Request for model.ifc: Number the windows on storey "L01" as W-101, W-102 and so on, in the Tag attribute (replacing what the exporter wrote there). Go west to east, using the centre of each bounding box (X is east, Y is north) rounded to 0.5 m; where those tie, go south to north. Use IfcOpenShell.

First a look at what the model holds.

```python
import ifcopenshell
import ifcopenshell.util.element
import ifcopenshell.util.placement

model = ifcopenshell.open("model.ifc")
print(model.schema)
storey = next(s for s in model.by_type("IfcBuildingStorey") if s.Name == "L01")
windows = [e for e in ifcopenshell.util.element.get_decomposition(storey) if e.is_a("IfcWindow")]
for e in sorted(windows, key=lambda e: e.id()):
    origin = ifcopenshell.util.placement.get_local_placement(e.ObjectPlacement)[:3, 3]
    print(e.id(), e.Tag, e.Name, origin.round(2) + 0.0, sep=" | ")
```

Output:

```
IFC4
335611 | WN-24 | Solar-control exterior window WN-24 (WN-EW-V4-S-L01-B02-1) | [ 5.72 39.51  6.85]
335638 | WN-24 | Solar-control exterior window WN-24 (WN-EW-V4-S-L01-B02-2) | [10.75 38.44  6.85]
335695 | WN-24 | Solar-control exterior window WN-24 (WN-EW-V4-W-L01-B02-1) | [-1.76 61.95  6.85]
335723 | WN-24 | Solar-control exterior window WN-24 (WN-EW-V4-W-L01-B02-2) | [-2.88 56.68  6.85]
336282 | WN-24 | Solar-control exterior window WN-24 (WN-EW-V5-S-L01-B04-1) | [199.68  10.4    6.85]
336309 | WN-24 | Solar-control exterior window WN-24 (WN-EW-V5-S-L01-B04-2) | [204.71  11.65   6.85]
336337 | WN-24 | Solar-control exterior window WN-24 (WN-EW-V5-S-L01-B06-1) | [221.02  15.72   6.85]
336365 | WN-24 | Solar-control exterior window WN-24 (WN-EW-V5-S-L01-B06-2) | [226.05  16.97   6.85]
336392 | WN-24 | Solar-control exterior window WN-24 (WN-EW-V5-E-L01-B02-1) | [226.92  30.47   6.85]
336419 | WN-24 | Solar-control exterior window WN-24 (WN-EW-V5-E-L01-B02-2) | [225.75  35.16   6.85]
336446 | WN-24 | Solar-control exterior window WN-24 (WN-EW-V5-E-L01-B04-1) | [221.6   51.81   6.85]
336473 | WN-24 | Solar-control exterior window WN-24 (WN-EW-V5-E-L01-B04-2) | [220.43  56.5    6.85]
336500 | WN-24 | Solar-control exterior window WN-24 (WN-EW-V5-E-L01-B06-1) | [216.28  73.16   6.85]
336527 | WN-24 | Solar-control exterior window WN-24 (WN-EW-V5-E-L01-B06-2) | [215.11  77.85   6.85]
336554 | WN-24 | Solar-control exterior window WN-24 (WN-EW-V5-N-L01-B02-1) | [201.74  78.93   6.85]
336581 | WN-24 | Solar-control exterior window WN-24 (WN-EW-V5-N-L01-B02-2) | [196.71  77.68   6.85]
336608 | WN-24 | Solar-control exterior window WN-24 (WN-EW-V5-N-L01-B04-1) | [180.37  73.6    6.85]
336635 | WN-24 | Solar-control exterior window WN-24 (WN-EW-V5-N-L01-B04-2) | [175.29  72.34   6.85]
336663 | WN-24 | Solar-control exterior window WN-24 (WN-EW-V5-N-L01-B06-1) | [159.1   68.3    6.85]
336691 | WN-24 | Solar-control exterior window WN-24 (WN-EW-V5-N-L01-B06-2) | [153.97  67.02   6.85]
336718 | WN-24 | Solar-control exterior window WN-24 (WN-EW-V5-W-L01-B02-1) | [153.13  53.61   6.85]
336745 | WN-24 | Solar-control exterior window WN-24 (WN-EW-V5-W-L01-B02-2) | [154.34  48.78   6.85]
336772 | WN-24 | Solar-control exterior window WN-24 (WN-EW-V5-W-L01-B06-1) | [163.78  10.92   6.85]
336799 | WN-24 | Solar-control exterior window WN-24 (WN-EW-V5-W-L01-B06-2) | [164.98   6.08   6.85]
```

```python
import ifcopenshell
import ifcopenshell.geom
import ifcopenshell.util.element
import ifcopenshell.util.shape

model = ifcopenshell.open("model.ifc")
settings = ifcopenshell.geom.settings()
settings.set("use-world-coords", True)


def centre(element):
    shape = ifcopenshell.geom.create_shape(settings, element)
    return ifcopenshell.util.shape.get_bbox_centroid(shape.geometry)


storey = next(s for s in model.by_type("IfcBuildingStorey") if s.Name == "L01")
windows = [e for e in ifcopenshell.util.element.get_decomposition(storey) if e.is_a("IfcWindow")]

# Insertion points can sit at a corner or the storey origin, so sort by the geometry (in metres).
centres = {e: centre(e) for e in windows}
windows.sort(key=lambda e: (round(centres[e][0] / 0.5), centres[e][1]))

for i, e in enumerate(windows, start=1):
    number = f"W-1{i:02d}"
    e.Tag = number
    print(e.id(), number)

model.write("model_edited.ifc")
```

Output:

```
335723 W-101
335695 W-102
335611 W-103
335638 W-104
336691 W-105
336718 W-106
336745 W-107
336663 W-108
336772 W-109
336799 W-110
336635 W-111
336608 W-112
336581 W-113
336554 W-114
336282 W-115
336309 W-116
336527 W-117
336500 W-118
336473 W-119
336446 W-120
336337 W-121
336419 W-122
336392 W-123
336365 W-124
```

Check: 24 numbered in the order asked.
